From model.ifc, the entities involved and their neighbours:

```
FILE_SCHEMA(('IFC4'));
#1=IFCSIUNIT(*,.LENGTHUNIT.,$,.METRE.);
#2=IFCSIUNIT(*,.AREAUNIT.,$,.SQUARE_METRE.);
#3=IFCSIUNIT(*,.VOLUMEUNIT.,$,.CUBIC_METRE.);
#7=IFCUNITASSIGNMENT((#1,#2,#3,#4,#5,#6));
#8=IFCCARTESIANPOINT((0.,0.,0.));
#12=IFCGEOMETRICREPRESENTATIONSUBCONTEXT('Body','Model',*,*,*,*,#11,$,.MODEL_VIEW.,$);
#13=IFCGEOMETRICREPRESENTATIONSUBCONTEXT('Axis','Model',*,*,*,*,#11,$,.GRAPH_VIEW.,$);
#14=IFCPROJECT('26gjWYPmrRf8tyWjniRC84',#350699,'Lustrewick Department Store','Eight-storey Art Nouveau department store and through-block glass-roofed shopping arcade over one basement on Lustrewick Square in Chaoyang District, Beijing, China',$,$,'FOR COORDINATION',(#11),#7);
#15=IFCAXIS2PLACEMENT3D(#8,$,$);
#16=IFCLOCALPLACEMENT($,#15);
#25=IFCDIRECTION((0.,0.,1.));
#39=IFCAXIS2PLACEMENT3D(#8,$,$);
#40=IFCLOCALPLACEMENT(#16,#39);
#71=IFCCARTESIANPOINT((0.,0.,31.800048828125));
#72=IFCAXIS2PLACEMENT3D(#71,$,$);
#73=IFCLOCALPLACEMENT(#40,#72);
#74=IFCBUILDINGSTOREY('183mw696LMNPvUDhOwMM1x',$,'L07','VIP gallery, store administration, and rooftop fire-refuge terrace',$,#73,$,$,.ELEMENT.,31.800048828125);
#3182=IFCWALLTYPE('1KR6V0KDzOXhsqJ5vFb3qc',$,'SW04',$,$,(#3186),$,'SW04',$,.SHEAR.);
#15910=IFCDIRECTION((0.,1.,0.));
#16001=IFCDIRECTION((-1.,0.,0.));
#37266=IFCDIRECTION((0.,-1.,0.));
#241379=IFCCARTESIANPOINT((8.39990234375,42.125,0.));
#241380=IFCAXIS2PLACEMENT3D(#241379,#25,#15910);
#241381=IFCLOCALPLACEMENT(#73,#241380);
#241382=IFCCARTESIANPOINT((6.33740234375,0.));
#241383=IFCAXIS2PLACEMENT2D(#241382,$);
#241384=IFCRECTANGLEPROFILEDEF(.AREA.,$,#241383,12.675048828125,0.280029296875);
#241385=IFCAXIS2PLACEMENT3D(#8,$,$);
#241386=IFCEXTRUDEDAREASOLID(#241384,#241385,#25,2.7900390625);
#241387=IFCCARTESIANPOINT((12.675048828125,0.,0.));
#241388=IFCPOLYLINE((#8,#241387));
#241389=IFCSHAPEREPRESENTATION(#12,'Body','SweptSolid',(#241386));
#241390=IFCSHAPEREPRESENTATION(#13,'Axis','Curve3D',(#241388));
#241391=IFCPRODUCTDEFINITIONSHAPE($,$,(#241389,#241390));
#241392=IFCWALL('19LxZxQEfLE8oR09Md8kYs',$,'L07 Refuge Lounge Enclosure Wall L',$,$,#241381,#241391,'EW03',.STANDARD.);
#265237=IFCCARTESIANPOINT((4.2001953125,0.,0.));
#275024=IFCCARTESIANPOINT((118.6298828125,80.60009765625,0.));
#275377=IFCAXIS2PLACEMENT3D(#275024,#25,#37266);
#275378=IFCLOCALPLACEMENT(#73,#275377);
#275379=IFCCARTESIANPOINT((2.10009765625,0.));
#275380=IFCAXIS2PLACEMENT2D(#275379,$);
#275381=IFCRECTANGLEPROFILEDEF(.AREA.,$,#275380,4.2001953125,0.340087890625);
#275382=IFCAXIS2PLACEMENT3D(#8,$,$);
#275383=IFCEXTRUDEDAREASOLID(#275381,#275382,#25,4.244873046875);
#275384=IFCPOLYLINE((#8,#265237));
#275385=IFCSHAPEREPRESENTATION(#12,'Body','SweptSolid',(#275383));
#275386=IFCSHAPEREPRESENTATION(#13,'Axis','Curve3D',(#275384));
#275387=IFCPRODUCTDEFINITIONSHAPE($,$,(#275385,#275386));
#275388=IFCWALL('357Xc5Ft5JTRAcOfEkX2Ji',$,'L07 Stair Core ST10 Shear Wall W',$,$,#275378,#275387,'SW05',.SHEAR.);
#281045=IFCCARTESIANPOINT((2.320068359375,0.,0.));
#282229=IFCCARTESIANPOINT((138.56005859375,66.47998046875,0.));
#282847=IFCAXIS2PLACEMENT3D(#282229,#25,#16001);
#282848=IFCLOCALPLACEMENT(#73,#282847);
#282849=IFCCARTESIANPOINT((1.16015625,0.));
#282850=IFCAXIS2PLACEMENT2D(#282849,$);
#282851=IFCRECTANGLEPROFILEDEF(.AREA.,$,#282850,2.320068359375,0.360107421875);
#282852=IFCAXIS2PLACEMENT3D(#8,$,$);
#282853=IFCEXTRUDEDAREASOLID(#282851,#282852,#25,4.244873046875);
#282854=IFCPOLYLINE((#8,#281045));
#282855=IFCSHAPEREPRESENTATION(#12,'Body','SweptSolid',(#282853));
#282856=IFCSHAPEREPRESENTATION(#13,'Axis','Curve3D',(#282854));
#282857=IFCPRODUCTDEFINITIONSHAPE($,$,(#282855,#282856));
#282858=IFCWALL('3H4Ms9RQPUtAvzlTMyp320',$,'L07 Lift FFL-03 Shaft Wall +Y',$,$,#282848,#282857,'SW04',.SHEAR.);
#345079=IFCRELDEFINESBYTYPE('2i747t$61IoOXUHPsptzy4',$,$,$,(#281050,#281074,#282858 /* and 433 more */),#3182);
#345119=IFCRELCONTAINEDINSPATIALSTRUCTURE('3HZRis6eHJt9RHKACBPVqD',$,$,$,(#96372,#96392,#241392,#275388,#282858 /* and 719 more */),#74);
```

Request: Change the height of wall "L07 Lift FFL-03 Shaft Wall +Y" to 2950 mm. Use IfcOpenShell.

```python
import ifcopenshell
import ifcopenshell.geom
import ifcopenshell.util.representation
import ifcopenshell.util.shape
import ifcopenshell.util.unit

model = ifcopenshell.open("model.ifc")
unit_scale = ifcopenshell.util.unit.calculate_unit_scale(model)
settings = ifcopenshell.geom.settings()


def volume(element):
    """Net volume in cubic metres, openings subtracted."""
    shape = ifcopenshell.geom.create_shape(settings, element)
    return ifcopenshell.util.shape.get_volume(shape.geometry)


wall = model.by_id(282858)
before = volume(wall)

body = ifcopenshell.util.representation.get_representation(wall, "Model", "Body")
solid = body.Items[0]
old_height = solid.Depth
solid.Depth = 2.95 / unit_scale
after = volume(wall)

print(f"height {old_height:g} -> {solid.Depth:g}, volume {before:.3f} -> {after:.3f} m3")

model.write("model_v2.ifc")
```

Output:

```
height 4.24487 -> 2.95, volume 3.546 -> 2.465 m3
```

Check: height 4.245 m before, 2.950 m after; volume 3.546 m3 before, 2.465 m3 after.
